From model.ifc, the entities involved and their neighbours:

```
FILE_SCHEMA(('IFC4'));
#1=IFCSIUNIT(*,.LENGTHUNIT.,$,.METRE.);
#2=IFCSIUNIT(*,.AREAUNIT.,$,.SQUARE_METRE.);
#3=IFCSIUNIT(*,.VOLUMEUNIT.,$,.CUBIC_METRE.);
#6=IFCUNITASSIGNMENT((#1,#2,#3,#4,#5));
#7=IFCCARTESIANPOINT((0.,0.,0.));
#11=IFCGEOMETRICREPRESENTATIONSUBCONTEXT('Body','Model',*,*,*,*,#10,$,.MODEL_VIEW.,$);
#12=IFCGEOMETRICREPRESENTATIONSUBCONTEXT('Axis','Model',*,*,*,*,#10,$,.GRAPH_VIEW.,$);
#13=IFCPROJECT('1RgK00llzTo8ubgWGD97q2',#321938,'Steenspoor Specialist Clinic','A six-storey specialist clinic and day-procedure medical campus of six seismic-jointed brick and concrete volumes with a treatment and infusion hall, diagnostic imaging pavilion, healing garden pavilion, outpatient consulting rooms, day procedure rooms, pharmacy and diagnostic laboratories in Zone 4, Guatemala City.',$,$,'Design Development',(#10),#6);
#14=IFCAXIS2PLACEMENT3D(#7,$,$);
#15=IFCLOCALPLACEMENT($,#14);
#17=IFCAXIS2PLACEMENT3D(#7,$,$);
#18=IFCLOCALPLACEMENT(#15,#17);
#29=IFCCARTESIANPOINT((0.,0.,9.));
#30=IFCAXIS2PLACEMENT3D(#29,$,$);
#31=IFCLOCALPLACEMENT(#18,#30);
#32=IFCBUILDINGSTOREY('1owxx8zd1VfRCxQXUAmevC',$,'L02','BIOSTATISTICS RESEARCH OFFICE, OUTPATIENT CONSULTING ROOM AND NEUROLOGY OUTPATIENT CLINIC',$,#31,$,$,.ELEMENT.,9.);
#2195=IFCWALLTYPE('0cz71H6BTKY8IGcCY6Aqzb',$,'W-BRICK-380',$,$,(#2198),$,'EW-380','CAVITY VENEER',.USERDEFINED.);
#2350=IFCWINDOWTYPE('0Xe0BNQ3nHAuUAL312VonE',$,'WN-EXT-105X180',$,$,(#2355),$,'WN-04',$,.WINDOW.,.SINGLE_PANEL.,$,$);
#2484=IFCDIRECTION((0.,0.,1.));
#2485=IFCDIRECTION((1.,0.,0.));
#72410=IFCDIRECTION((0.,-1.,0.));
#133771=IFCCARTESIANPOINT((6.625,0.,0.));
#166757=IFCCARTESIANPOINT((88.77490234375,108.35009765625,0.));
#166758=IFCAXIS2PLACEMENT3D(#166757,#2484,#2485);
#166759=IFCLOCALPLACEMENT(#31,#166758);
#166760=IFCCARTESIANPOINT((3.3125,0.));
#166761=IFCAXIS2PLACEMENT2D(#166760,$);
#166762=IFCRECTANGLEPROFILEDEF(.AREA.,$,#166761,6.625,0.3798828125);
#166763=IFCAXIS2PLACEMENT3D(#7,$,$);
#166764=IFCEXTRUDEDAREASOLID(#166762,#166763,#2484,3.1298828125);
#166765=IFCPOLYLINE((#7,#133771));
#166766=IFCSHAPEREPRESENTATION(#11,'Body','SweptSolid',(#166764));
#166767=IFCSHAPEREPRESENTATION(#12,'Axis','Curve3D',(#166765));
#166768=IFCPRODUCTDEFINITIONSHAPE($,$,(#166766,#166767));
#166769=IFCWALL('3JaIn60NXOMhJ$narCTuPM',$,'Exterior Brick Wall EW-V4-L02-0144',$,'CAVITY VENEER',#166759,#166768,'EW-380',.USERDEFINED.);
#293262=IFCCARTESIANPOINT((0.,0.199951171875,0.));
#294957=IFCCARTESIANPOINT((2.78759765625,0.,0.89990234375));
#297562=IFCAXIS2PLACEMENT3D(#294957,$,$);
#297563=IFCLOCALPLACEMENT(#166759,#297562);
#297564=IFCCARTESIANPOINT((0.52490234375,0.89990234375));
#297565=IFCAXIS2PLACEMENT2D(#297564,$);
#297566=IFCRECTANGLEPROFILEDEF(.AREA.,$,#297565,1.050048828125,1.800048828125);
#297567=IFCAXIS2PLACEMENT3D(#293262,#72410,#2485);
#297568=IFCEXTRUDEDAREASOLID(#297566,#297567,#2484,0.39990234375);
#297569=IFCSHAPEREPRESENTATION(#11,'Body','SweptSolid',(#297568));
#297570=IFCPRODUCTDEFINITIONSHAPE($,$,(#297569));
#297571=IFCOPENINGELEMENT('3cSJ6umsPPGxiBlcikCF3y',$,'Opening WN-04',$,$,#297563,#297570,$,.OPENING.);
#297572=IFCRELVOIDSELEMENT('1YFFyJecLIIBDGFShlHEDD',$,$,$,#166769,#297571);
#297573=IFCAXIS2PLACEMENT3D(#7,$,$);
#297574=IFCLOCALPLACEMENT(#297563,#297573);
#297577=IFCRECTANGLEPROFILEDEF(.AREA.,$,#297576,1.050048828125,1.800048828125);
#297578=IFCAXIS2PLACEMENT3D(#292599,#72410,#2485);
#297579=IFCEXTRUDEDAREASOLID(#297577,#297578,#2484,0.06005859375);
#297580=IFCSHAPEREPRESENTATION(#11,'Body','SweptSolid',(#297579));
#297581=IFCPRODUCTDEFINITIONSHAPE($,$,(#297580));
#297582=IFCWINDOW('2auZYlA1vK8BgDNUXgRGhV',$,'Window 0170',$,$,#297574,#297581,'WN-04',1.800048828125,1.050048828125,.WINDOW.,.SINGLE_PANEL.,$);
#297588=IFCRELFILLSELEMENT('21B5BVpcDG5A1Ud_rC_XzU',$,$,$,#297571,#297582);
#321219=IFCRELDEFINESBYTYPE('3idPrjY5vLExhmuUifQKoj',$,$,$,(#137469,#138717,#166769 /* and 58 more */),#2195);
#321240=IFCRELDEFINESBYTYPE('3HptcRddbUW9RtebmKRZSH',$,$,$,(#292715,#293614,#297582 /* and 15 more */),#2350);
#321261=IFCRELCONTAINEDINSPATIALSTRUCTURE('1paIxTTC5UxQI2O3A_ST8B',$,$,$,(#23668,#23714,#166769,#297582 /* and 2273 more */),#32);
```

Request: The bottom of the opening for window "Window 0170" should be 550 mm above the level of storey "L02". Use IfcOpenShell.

```python
import numpy as np
import ifcopenshell
import ifcopenshell.api.geometry
import ifcopenshell.geom
import ifcopenshell.util.element
import ifcopenshell.util.placement
import ifcopenshell.util.shape
import ifcopenshell.util.unit

model = ifcopenshell.open("model.ifc")
unit_scale = ifcopenshell.util.unit.calculate_unit_scale(model)

window = model.by_guid("2auZYlA1vK8BgDNUXgRGhV")
opening = window.FillsVoids[0].RelatingOpeningElement
storey = ifcopenshell.util.element.get_container(window, ifc_class="IfcBuildingStorey")
level = ifcopenshell.util.placement.get_local_placement(storey.ObjectPlacement)[2, 3]

# The opening's origin need not be at the sill, so measure its lowest point.
shape = ifcopenshell.geom.create_shape(ifcopenshell.geom.settings(), opening)
bottom = ifcopenshell.util.shape.get_shape_bottom_elevation(shape, shape.geometry) / unit_scale
dz = level + 0.55 - bottom

shift = np.array([0.0, 0.0, dz])
# The window is placed relative to its opening, so it follows when the opening moves.
matrix = ifcopenshell.util.placement.get_local_placement(opening.ObjectPlacement)
matrix[:3, 3] += shift
ifcopenshell.api.geometry.edit_object_placement(
    model, product=opening, matrix=matrix, is_si=False, should_transform_children=True
)

print(f"moved by {dz * unit_scale:+.3f} m")

model.write("model_updated.ifc")
```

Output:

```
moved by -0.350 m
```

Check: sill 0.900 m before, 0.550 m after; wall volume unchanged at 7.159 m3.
